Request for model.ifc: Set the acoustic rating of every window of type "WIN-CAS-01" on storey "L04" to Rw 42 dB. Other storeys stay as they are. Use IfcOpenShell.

First a look at what the model holds.

```python
import ifcopenshell
import ifcopenshell.util.element

model = ifcopenshell.open("model.ifc")
print(model.schema)
storey = next(s for s in model.by_type("IfcBuildingStorey") if s.Name == "L04")
windows = [e for e in ifcopenshell.util.element.get_decomposition(storey) if e.is_a("IfcWindow")]
seen = {}
for e in windows:
    element_type = ifcopenshell.util.element.get_type(e)
    key = (element_type.Name if element_type != e and element_type else None, ifcopenshell.util.element.get_pset(e, "Pset_WindowCommon", "AcousticRating"))
    seen[key] = seen.get(key, 0) + 1
for (name, value), count in sorted(seen.items(), key=str):
    print(count, "x", name, "|", value)
```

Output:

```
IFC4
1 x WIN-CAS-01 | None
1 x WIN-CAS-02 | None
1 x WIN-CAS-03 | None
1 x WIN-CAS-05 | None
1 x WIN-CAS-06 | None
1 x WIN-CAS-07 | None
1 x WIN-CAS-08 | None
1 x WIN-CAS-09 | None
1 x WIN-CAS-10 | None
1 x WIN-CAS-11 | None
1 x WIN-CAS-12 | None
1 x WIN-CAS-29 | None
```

```python
import ifcopenshell
import ifcopenshell.api.pset
import ifcopenshell.util.element

model = ifcopenshell.open("model.ifc")

storey = next(s for s in model.by_type("IfcBuildingStorey") if s.Name == "L04")
windows = [e for e in ifcopenshell.util.element.get_decomposition(storey) if e.is_a("IfcWindow")]

count = 0
for e in windows:
    element_type = ifcopenshell.util.element.get_type(e)
    if element_type in (None, e) or element_type.Name != "WIN-CAS-01":
        continue
    # add_pset returns the element's existing set when there is one.
    pset = ifcopenshell.api.pset.add_pset(model, product=e, name="Pset_WindowCommon")
    ifcopenshell.api.pset.edit_pset(model, pset=pset, properties={"AcousticRating": "Rw 42 dB"})
    count += 1

print(count, "windows updated")

model.write("model_updated.ifc")
```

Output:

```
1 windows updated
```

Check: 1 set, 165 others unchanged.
